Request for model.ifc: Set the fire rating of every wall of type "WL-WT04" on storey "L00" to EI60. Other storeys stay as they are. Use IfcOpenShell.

First a look at what the model holds.

```python
import ifcopenshell
import ifcopenshell.util.element

model = ifcopenshell.open("model.ifc")
print(model.schema)
storey = next(s for s in model.by_type("IfcBuildingStorey") if s.Name == "L00")
walls = [e for e in ifcopenshell.util.element.get_decomposition(storey) if e.is_a("IfcWall")]
seen = {}
for e in walls:
    element_type = ifcopenshell.util.element.get_type(e)
    key = (element_type.Name if element_type != e and element_type else None, ifcopenshell.util.element.get_pset(e, "Pset_WallCommon", "FireRating"))
    seen[key] = seen.get(key, 0) + 1
for (name, value), count in sorted(seen.items(), key=str):
    print(count, "x", name, "|", value)
```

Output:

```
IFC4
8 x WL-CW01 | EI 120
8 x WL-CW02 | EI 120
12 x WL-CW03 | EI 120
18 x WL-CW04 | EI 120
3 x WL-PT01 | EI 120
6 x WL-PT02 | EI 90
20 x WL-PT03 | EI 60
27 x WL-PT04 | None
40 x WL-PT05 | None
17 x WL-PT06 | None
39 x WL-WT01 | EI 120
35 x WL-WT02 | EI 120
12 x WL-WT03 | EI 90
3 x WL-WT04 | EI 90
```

```python
import ifcopenshell
import ifcopenshell.api.pset
import ifcopenshell.util.element

model = ifcopenshell.open("model.ifc")

storey = next(s for s in model.by_type("IfcBuildingStorey") if s.Name == "L00")
walls = [e for e in ifcopenshell.util.element.get_decomposition(storey) if e.is_a("IfcWall")]

count = 0
for e in walls:
    element_type = ifcopenshell.util.element.get_type(e)
    if element_type in (None, e) or element_type.Name != "WL-WT04":
        continue
    # add_pset returns the element's existing set when there is one.
    pset = ifcopenshell.api.pset.add_pset(model, product=e, name="Pset_WallCommon")
    ifcopenshell.api.pset.edit_pset(model, pset=pset, properties={"FireRating": "EI60"})
    count += 1

print(count, "walls updated")

model.write("model_edited.ifc")
```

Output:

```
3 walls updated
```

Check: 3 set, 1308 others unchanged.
